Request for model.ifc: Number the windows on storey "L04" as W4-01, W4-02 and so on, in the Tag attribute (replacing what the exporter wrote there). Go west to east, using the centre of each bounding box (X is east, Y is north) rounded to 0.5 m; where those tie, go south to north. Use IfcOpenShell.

First a look at what the model holds.

```python
import ifcopenshell
import ifcopenshell.util.element
import ifcopenshell.util.placement

model = ifcopenshell.open("model.ifc")
print(model.schema)
storey = next(s for s in model.by_type("IfcBuildingStorey") if s.Name == "L04")
windows = [e for e in ifcopenshell.util.element.get_decomposition(storey) if e.is_a("IfcWindow")]
for e in sorted(windows, key=lambda e: e.id()):
    origin = ifcopenshell.util.placement.get_local_placement(e.ObjectPlacement)[:3, 3]
    print(e.id(), e.Tag, e.Name, origin.round(2) + 0.0, sep=" | ")
```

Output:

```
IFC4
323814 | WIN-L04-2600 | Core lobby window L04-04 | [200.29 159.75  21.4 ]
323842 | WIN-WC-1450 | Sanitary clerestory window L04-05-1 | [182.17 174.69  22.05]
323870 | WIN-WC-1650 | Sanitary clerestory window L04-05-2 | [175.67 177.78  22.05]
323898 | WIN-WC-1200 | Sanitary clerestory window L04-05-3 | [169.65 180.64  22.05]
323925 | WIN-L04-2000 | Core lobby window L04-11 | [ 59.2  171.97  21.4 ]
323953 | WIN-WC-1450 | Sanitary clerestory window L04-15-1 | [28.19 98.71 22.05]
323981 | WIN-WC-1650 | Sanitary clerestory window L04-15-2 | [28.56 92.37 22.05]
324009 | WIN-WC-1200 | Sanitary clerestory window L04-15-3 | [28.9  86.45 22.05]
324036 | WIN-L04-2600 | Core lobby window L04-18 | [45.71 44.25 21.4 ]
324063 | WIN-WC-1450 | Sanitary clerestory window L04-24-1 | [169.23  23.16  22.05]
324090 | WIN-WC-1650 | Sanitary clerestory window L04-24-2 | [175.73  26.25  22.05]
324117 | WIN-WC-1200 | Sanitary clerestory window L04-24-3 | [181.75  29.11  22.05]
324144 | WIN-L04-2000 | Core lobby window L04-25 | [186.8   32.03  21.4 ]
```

```python
import ifcopenshell
import ifcopenshell.geom
import ifcopenshell.util.element
import ifcopenshell.util.shape

model = ifcopenshell.open("model.ifc")
settings = ifcopenshell.geom.settings()
settings.set("use-world-coords", True)


def centre(element):
    shape = ifcopenshell.geom.create_shape(settings, element)
    return ifcopenshell.util.shape.get_bbox_centroid(shape.geometry)


storey = next(s for s in model.by_type("IfcBuildingStorey") if s.Name == "L04")
windows = [e for e in ifcopenshell.util.element.get_decomposition(storey) if e.is_a("IfcWindow")]

# Insertion points can sit at a corner or the storey origin, so sort by the geometry (in metres).
centres = {e: centre(e) for e in windows}
windows.sort(key=lambda e: (round(centres[e][0] / 0.5), centres[e][1]))

for i, e in enumerate(windows, start=1):
    number = f"W4-{i:02d}"
    e.Tag = number
    print(e.id(), number)

model.write("model_edited.ifc")
```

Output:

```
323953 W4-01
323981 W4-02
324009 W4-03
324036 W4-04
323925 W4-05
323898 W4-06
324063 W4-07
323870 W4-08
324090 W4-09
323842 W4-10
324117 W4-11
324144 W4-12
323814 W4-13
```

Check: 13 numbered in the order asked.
